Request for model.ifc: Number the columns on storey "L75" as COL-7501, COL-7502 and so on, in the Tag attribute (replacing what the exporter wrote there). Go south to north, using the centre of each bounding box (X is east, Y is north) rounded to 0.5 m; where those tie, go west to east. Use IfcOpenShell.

First a look at what the model holds.

```python
import ifcopenshell
import ifcopenshell.util.element
import ifcopenshell.util.placement

model = ifcopenshell.open("model.ifc")
print(model.schema)
storey = next(s for s in model.by_type("IfcBuildingStorey") if s.Name == "L75")
columns = [e for e in ifcopenshell.util.element.get_decomposition(storey) if e.is_a("IfcColumn")]
for e in sorted(columns, key=lambda e: e.id()):
    origin = ifcopenshell.util.placement.get_local_placement(e.ObjectPlacement)[:3, 3]
    print(e.id(), e.Tag, e.Name, origin.round(2) + 0.0, sep=" | ")
```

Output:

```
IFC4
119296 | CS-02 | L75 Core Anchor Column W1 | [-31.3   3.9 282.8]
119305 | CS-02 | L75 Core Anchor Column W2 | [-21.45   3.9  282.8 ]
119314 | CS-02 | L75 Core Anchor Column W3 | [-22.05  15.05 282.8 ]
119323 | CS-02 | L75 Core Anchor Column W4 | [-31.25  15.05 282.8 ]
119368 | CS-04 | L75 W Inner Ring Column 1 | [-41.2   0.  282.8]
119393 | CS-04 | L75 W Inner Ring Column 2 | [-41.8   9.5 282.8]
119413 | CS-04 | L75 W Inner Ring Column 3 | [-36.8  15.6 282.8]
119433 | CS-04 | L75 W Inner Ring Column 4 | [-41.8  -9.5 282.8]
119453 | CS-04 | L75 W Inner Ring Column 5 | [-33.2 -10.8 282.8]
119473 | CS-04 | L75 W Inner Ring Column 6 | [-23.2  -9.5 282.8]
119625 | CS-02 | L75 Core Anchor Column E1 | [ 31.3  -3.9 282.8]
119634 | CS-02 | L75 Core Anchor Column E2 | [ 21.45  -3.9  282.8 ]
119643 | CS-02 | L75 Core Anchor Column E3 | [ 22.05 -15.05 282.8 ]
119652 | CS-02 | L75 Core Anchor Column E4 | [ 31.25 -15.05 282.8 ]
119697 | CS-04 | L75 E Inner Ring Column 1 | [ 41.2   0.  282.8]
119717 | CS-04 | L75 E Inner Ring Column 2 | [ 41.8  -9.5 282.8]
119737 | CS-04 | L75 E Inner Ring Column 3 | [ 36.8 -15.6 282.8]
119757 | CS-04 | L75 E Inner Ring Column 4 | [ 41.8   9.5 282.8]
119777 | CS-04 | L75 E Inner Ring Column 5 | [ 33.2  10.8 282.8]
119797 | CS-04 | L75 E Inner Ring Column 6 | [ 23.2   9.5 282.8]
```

```python
import ifcopenshell
import ifcopenshell.geom
import ifcopenshell.util.element
import ifcopenshell.util.shape

model = ifcopenshell.open("model.ifc")
settings = ifcopenshell.geom.settings()
settings.set("use-world-coords", True)


def centre(element):
    shape = ifcopenshell.geom.create_shape(settings, element)
    return ifcopenshell.util.shape.get_bbox_centroid(shape.geometry)


storey = next(s for s in model.by_type("IfcBuildingStorey") if s.Name == "L75")
columns = [e for e in ifcopenshell.util.element.get_decomposition(storey) if e.is_a("IfcColumn")]

# Insertion points can sit at a corner or the storey origin, so sort by the geometry (in metres).
centres = {e: centre(e) for e in columns}
columns.sort(key=lambda e: (round(centres[e][1] / 0.5), centres[e][0]))

for i, e in enumerate(columns, start=1):
    number = f"COL-75{i:02d}"
    e.Tag = number
    print(e.id(), number)

model.write("model_edited.ifc")
```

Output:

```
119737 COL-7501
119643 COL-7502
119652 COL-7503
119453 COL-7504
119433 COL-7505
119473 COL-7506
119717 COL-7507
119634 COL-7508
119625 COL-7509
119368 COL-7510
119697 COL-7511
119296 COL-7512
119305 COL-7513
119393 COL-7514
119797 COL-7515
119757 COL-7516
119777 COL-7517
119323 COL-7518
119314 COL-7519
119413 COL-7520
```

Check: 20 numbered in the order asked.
